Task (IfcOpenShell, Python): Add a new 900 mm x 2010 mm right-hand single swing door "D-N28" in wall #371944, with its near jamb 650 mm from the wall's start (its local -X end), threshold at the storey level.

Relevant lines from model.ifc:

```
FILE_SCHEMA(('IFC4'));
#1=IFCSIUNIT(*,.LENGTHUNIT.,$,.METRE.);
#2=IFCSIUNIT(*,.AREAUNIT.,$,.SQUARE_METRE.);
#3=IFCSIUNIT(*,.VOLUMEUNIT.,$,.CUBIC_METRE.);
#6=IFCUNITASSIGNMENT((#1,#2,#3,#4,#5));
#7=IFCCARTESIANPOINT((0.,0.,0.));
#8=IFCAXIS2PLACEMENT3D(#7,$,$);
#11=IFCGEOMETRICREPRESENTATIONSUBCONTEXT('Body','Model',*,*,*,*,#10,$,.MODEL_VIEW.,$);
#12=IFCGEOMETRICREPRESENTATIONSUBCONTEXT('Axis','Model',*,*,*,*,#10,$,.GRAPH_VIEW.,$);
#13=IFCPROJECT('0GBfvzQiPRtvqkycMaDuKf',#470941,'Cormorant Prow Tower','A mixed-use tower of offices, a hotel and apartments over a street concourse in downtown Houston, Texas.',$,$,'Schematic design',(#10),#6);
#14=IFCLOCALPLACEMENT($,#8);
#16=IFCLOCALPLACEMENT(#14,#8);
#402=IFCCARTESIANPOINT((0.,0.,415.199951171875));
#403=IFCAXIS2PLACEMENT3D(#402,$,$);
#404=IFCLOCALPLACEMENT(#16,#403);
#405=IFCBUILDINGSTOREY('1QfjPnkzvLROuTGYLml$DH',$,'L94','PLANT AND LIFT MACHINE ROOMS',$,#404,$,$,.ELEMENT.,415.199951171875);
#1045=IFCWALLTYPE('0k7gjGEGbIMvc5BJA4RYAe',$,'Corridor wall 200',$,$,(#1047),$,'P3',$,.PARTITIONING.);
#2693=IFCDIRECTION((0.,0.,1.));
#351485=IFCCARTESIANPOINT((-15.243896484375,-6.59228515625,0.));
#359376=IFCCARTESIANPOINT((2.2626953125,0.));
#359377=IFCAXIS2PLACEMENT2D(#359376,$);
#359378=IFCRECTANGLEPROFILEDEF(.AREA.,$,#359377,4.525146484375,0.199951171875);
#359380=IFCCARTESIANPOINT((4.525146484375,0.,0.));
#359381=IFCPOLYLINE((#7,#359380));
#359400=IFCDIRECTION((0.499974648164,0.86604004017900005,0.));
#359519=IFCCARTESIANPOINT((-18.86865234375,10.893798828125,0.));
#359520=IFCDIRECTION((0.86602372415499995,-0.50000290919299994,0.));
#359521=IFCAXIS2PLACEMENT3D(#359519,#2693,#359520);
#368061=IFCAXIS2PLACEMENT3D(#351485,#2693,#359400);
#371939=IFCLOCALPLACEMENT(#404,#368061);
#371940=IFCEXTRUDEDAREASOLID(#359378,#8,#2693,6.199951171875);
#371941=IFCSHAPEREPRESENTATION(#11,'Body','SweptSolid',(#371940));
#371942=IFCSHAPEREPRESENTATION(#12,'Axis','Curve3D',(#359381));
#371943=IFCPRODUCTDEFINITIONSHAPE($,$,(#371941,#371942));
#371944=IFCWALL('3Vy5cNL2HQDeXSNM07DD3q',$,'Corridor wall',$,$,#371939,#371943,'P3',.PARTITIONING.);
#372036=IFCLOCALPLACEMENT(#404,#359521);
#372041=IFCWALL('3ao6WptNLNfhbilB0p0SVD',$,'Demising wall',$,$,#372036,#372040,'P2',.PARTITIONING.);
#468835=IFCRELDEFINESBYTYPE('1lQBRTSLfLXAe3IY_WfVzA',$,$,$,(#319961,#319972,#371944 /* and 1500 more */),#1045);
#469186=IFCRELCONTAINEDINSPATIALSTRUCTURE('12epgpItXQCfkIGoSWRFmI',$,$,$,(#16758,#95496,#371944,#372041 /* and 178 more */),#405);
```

```python
import numpy as np
import ifcopenshell
import ifcopenshell.api.feature
import ifcopenshell.api.geometry
import ifcopenshell.api.root
import ifcopenshell.api.spatial
import ifcopenshell.geom
import ifcopenshell.util.element
import ifcopenshell.util.placement
import ifcopenshell.util.representation
import ifcopenshell.util.shape
import ifcopenshell.util.unit

model = ifcopenshell.open("model.ifc")
unit_scale = ifcopenshell.util.unit.calculate_unit_scale(model)
settings = ifcopenshell.geom.settings()


def volume(element):
    """Net volume in cubic metres, openings subtracted."""
    shape = ifcopenshell.geom.create_shape(settings, element)
    return ifcopenshell.util.shape.get_volume(shape.geometry)


wall = model.by_guid("3Vy5cNL2HQDeXSNM07DD3q")
storey = ifcopenshell.util.element.get_container(wall, ifc_class="IfcBuildingStorey")
context = ifcopenshell.util.representation.get_context(model, "Model", "Body", "MODEL_VIEW")
before = volume(wall)

width, height, from_end, sill = 0.9, 2.01, 0.65, 0.0  # metres

# The wall runs along its own X axis, and the end named is its -X end.
wall_shape = ifcopenshell.geom.create_shape(settings, wall)
x, y, z = ifcopenshell.util.shape.get_vertices(wall_shape.geometry).T
start = x.min() + from_end
face, thickness = float(y.min()), float(y.max() - y.min())
wall_matrix = ifcopenshell.util.placement.get_local_placement(wall.ObjectPlacement)
level = ifcopenshell.util.placement.get_local_placement(storey.ObjectPlacement)[2, 3]


def in_wall(x, y):
    """Placement at x, y metres in the wall's axes, at sill height."""
    matrix = wall_matrix.copy()
    matrix[:, 3] = wall_matrix @ np.array([x / unit_scale, y / unit_scale, 0.0, 1.0])
    matrix[2, 3] = level + sill / unit_scale
    return matrix


# Opening: a box that overshoots both wall faces by 50 mm.
opening = ifcopenshell.api.root.create_entity(model, ifc_class="IfcOpeningElement", predefined_type="OPENING")
box = ifcopenshell.api.geometry.add_wall_representation(
    model, context=context, length=width, height=height, thickness=thickness + 0.1
)
ifcopenshell.api.geometry.assign_representation(model, product=opening, representation=box)
ifcopenshell.api.geometry.edit_object_placement(model, product=opening, matrix=in_wall(start, face - 0.05), is_si=False)
ifcopenshell.api.feature.add_feature(model, feature=opening, element=wall)

door = ifcopenshell.api.root.create_entity(model, ifc_class="IfcDoor", name="D-N28", predefined_type="DOOR")
door.OverallWidth, door.OverallHeight = width / unit_scale, height / unit_scale
door.OperationType = "SINGLE_SWING_RIGHT"
body = ifcopenshell.api.geometry.add_door_representation(
    model,
    context=context,
    overall_width=door.OverallWidth,
    overall_height=door.OverallHeight,
    operation_type="SINGLE_SWING_RIGHT",
    lining_properties={"LiningDepth": thickness / unit_scale, "ThresholdDepth": thickness / unit_scale},
)
ifcopenshell.api.geometry.assign_representation(model, product=door, representation=body)
ifcopenshell.api.spatial.assign_container(model, products=[door], relating_structure=storey)
ifcopenshell.api.feature.add_filling(model, opening=opening, element=door)

# The lining spans the wall, so the door starts at the wall face.
ifcopenshell.api.geometry.edit_object_placement(model, product=door, matrix=in_wall(start, face), is_si=False)

after = volume(wall)

print(f"wall volume {before:.3f} -> {after:.3f} m3")

model.write("model_edited.ifc")
```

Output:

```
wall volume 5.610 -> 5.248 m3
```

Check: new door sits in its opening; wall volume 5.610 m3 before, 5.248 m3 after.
